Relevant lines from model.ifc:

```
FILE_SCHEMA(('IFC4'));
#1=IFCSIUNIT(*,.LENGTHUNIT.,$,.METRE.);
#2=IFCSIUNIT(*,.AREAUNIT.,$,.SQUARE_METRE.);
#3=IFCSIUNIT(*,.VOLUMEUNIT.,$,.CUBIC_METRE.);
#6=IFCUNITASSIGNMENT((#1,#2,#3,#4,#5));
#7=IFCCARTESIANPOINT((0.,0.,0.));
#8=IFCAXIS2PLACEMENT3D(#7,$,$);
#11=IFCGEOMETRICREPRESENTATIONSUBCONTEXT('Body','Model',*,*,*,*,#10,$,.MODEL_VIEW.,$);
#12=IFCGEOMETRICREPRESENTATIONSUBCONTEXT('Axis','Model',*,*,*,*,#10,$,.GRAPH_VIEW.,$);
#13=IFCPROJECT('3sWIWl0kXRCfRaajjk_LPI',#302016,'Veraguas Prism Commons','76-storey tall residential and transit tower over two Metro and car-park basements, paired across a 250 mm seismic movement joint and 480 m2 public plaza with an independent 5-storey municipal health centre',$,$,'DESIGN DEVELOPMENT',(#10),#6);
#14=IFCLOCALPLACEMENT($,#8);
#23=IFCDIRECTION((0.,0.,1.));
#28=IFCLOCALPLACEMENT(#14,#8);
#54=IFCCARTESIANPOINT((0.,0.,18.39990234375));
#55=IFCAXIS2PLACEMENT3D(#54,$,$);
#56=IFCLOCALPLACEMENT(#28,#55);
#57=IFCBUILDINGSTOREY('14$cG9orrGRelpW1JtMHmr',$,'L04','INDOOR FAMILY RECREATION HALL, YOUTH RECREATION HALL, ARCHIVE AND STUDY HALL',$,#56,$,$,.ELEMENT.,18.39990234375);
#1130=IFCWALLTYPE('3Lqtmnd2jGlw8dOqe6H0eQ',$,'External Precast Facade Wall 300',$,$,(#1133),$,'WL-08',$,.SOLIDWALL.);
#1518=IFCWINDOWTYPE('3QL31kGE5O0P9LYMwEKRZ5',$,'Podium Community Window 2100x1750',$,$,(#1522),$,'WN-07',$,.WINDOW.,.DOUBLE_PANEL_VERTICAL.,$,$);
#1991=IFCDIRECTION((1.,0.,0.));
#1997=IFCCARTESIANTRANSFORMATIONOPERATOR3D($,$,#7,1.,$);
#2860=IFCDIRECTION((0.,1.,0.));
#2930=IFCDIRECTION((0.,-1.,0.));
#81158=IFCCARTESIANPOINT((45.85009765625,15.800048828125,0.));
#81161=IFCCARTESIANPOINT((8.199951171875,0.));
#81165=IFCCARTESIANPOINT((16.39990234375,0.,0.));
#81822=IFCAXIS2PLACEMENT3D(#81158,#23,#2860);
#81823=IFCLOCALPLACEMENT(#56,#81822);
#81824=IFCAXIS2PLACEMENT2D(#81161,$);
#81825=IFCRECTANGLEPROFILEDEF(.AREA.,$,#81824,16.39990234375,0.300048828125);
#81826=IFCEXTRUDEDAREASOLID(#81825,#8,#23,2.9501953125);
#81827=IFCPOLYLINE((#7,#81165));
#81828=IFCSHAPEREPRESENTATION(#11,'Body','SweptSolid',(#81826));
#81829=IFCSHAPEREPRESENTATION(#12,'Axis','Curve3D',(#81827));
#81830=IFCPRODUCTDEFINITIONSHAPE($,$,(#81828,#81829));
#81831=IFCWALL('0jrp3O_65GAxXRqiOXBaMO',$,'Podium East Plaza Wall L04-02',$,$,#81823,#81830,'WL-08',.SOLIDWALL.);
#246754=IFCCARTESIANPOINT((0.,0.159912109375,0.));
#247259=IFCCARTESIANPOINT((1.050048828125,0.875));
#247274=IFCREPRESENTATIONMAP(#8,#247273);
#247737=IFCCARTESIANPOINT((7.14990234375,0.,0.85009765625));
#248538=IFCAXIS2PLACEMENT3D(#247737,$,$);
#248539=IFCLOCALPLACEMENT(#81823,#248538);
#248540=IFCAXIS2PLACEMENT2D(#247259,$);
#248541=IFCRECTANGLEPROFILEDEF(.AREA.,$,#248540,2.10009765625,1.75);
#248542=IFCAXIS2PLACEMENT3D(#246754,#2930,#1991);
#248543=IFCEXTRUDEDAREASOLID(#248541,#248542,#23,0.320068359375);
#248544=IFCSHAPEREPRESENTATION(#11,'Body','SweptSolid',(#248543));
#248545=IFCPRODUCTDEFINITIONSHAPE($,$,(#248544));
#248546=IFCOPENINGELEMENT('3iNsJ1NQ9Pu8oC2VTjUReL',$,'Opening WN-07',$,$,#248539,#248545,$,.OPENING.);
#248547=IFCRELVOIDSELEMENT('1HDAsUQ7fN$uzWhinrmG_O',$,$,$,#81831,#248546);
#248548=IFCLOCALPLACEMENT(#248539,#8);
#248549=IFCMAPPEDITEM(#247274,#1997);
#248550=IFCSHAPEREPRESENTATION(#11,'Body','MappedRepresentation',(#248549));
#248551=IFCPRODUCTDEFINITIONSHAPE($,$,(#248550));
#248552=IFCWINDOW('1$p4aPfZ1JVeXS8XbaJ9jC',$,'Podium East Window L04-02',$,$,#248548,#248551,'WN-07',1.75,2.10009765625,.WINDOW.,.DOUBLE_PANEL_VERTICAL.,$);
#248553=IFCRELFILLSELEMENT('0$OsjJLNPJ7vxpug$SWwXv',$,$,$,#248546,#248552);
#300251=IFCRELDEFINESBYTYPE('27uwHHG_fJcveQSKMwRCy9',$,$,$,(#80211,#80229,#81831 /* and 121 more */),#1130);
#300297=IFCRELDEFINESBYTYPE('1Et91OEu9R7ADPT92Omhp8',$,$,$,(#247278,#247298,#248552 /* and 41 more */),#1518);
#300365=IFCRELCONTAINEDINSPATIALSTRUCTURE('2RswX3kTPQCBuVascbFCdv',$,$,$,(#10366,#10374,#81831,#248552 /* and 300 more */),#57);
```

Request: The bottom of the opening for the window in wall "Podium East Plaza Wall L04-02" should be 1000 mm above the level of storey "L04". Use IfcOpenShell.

```python
import numpy as np
import ifcopenshell
import ifcopenshell.api.geometry
import ifcopenshell.geom
import ifcopenshell.util.element
import ifcopenshell.util.placement
import ifcopenshell.util.shape
import ifcopenshell.util.unit

model = ifcopenshell.open("model.ifc")
unit_scale = ifcopenshell.util.unit.calculate_unit_scale(model)

window = model.by_guid("1$p4aPfZ1JVeXS8XbaJ9jC")
opening = window.FillsVoids[0].RelatingOpeningElement
storey = ifcopenshell.util.element.get_container(window, ifc_class="IfcBuildingStorey")
level = ifcopenshell.util.placement.get_local_placement(storey.ObjectPlacement)[2, 3]

# The opening's origin need not be at the sill, so measure its lowest point.
shape = ifcopenshell.geom.create_shape(ifcopenshell.geom.settings(), opening)
bottom = ifcopenshell.util.shape.get_shape_bottom_elevation(shape, shape.geometry) / unit_scale
dz = level + 1 / unit_scale - bottom

shift = np.array([0.0, 0.0, dz])
# The window is placed relative to its opening, so it follows when the opening moves.
matrix = ifcopenshell.util.placement.get_local_placement(opening.ObjectPlacement)
matrix[:3, 3] += shift
ifcopenshell.api.geometry.edit_object_placement(
    model, product=opening, matrix=matrix, is_si=False, should_transform_children=True
)

print(f"moved by {dz * unit_scale:+.3f} m")

model.write("model_updated.ifc")
```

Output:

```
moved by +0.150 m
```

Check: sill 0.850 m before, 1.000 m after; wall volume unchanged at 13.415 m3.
